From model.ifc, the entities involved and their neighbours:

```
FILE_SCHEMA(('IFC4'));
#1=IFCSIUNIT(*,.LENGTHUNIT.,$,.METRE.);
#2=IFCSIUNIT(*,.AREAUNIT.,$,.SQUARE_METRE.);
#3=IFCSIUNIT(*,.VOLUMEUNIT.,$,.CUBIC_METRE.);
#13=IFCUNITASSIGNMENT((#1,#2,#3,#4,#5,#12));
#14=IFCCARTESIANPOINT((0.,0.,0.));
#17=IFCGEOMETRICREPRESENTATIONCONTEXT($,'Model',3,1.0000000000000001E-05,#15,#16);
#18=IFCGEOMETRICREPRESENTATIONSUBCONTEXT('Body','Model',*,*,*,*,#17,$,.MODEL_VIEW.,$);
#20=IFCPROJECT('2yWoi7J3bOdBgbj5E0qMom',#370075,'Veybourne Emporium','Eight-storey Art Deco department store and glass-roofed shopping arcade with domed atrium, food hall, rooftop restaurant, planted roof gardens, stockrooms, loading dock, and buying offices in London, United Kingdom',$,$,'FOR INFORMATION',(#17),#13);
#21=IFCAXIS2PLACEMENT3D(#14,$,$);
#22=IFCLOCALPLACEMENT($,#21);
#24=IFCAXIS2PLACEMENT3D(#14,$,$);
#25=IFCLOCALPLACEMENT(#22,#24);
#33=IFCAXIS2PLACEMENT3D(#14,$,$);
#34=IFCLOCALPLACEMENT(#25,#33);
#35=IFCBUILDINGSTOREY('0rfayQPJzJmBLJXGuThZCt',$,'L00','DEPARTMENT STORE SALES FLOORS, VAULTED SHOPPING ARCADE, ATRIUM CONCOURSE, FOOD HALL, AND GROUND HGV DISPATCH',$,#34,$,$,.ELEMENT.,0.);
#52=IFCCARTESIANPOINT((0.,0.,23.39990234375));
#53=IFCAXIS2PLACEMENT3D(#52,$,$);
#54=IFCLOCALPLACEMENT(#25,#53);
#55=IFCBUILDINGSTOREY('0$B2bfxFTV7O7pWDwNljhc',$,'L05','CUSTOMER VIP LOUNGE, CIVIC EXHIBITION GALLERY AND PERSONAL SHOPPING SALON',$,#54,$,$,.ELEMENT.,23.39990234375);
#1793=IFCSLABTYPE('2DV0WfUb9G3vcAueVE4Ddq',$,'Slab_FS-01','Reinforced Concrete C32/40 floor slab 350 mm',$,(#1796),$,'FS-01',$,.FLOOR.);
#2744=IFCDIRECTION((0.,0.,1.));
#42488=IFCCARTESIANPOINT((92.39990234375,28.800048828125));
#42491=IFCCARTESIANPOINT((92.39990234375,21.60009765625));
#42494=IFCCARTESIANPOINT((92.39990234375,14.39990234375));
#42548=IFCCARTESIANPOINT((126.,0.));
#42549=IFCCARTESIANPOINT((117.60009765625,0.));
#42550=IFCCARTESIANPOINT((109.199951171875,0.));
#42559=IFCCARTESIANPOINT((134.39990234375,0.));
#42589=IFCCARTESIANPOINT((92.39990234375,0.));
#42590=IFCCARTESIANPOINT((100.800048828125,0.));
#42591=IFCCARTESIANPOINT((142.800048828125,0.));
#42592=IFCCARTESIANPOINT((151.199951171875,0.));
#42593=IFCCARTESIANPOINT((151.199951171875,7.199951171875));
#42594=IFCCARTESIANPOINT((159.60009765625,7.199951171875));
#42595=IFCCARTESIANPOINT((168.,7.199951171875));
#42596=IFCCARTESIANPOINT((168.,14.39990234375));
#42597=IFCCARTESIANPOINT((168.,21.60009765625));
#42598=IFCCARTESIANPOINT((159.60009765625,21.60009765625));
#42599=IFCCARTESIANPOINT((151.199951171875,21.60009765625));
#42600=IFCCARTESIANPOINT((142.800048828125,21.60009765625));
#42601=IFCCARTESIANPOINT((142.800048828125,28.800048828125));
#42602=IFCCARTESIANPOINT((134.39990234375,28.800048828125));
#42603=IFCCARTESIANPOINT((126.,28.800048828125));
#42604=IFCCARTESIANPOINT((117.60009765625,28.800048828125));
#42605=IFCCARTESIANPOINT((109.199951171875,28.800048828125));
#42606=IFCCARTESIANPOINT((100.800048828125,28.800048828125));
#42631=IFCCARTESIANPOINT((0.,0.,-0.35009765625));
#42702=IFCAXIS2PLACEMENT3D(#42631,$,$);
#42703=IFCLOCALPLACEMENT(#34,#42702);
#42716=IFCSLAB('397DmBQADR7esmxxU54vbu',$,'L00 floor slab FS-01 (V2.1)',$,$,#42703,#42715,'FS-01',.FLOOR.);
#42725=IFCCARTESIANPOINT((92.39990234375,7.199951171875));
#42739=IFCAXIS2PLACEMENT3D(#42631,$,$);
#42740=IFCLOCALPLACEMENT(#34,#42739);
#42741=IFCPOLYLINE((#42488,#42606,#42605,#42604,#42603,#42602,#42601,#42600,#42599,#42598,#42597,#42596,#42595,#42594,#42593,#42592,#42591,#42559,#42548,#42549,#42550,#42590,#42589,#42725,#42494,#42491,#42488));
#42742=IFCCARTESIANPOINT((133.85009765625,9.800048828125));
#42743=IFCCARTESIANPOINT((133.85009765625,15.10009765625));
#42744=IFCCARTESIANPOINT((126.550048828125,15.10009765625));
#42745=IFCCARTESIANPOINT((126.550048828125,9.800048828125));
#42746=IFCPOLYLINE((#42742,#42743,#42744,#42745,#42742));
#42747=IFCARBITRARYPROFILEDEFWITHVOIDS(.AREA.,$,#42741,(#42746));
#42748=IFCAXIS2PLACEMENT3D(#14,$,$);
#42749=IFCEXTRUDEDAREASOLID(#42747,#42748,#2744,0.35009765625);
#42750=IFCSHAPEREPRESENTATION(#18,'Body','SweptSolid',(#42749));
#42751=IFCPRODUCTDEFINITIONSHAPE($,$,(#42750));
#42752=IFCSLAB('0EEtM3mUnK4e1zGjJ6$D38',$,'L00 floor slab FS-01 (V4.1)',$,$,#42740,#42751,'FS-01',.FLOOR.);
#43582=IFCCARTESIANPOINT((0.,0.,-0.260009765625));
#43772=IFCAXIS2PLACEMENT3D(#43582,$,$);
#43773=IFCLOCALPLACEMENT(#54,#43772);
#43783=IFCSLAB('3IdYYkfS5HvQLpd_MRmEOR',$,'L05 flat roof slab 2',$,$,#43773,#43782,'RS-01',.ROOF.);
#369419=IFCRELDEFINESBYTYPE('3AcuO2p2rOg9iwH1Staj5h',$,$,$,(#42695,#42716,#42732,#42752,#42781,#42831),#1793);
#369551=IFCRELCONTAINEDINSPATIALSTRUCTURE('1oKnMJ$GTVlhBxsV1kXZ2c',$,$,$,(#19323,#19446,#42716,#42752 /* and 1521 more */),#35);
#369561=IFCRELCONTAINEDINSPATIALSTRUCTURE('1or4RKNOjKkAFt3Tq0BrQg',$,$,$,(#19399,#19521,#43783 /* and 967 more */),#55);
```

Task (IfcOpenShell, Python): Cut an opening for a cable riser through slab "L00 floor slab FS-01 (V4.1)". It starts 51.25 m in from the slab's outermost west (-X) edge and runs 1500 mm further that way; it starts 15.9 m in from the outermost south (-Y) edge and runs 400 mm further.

```python
import numpy as np
import ifcopenshell
import ifcopenshell.api.feature
import ifcopenshell.api.geometry
import ifcopenshell.api.root
import ifcopenshell.geom
import ifcopenshell.util.placement
import ifcopenshell.util.representation
import ifcopenshell.util.shape
import ifcopenshell.util.unit

model = ifcopenshell.open("model.ifc")
unit_scale = ifcopenshell.util.unit.calculate_unit_scale(model)
settings = ifcopenshell.geom.settings()


def volume(element):
    """Net volume in cubic metres, openings subtracted."""
    shape = ifcopenshell.geom.create_shape(settings, element)
    return ifcopenshell.util.shape.get_volume(shape.geometry)


slab = model.by_id(42752)
before = volume(slab)

# Extent in the slab's own axes, in metres. The edges named are its -X and -Y sides.
slab_shape = ifcopenshell.geom.create_shape(settings, slab)
vertices = ifcopenshell.util.shape.get_vertices(slab_shape.geometry)
x_min, y_min, bottom = vertices.min(axis=0)
top = vertices[:, 2].max()

opening = ifcopenshell.api.root.create_entity(model, ifc_class="IfcOpeningElement", name="Cable riser opening", predefined_type="OPENING")
context = ifcopenshell.util.representation.get_context(model, "Model", "Body", "MODEL_VIEW")
width, depth = 1.5, 0.4
outline = [(0.0, 0.0), (width, 0.0), (width, depth), (0.0, depth), (0.0, 0.0)]
# Overshoot both faces by 50 mm so the cut is clean.
shape = ifcopenshell.api.geometry.add_slab_representation(
    model, context=context, depth=top - bottom + 0.1, polyline=outline
)
ifcopenshell.api.geometry.assign_representation(model, product=opening, representation=shape)

matrix = ifcopenshell.util.placement.get_local_placement(slab.ObjectPlacement)
matrix[:, 3] = matrix @ np.append(np.array([x_min + 51.25, y_min + 15.9, bottom - 0.05]) / unit_scale, 1.0)
ifcopenshell.api.geometry.edit_object_placement(model, product=opening, matrix=matrix, is_si=False)
ifcopenshell.api.feature.add_feature(model, feature=opening, element=slab)

after = volume(slab)

print(f"slab volume {before:.3f} -> {after:.3f} m3")

model.write("model_rev.ifc")
```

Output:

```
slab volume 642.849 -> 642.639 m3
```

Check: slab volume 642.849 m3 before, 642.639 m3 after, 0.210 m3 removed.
